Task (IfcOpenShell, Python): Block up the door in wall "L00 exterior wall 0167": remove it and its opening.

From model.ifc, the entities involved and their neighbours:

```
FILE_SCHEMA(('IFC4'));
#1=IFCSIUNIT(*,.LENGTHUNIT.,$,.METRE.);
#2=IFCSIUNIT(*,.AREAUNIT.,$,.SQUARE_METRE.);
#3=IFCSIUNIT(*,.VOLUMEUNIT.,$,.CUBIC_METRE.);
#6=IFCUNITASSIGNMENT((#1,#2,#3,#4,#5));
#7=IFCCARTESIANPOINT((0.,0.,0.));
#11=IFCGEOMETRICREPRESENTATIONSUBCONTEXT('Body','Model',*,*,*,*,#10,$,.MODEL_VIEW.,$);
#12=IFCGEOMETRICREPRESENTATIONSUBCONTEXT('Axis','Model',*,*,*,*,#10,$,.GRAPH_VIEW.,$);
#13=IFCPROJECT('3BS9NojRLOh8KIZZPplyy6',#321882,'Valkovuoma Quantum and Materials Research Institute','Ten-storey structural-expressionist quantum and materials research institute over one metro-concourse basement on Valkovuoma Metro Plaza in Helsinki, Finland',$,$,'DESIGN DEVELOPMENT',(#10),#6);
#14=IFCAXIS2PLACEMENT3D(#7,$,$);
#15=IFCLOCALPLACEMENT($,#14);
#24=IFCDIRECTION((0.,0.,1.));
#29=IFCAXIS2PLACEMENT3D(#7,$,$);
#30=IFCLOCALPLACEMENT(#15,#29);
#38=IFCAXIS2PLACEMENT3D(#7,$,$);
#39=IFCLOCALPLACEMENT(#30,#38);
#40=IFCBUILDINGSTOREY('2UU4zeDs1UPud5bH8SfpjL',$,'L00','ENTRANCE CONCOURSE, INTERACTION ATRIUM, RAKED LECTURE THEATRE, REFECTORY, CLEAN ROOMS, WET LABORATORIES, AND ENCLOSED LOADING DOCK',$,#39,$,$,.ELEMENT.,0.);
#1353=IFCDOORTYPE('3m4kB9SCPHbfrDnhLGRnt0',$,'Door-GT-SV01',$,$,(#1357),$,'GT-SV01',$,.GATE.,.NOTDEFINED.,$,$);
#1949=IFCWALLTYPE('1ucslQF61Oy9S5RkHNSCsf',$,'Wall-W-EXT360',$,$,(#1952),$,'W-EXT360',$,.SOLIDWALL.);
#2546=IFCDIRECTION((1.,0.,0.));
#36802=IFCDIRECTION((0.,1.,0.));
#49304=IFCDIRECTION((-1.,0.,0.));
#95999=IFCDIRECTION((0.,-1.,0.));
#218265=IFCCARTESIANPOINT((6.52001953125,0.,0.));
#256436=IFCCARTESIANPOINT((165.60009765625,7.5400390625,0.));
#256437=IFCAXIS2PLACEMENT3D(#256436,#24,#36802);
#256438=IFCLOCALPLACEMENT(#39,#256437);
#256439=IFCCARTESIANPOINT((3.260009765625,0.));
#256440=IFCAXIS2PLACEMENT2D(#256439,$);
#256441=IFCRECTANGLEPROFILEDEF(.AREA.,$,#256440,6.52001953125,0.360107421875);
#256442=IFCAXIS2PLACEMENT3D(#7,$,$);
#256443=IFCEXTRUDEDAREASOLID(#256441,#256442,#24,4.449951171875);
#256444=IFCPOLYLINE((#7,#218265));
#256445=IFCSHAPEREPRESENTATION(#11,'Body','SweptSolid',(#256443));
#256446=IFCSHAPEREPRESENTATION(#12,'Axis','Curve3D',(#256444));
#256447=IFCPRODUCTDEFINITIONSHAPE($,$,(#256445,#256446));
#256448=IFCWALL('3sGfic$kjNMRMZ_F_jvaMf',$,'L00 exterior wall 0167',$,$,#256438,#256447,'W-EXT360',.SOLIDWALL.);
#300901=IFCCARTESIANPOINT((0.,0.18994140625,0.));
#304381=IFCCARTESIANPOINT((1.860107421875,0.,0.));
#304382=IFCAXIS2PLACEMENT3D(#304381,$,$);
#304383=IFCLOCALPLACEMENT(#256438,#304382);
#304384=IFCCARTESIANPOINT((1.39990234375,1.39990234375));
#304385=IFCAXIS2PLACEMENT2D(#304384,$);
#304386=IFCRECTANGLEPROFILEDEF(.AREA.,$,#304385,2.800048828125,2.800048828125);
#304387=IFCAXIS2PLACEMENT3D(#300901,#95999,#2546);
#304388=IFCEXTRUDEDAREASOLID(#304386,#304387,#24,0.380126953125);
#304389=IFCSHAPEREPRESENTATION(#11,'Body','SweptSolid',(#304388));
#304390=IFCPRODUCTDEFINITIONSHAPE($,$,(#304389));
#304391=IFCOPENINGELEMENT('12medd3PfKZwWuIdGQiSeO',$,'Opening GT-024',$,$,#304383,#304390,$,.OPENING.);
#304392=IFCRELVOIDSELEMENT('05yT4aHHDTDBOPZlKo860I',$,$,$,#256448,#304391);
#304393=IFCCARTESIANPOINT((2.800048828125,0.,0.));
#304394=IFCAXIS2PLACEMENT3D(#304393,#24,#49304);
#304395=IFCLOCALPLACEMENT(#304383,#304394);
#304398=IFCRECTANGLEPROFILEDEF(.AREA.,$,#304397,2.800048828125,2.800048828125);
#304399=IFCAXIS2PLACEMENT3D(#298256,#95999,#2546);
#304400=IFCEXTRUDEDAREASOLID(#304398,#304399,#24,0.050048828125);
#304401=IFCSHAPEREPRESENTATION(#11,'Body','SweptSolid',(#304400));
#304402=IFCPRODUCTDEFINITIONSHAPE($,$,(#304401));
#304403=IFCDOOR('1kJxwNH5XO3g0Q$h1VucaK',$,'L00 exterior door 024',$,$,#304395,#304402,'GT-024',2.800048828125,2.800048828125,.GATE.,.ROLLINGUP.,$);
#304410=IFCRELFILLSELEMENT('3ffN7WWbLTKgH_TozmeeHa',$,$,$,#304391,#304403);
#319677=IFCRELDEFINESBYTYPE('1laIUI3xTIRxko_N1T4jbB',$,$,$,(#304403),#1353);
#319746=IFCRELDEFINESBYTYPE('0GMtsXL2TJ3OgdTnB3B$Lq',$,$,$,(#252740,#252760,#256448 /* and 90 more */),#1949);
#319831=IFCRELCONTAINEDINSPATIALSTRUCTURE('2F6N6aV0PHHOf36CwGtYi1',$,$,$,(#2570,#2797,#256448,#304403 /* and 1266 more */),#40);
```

```python
import ifcopenshell
import ifcopenshell.api.feature
import ifcopenshell.api.root
import ifcopenshell.geom
import ifcopenshell.util.shape

model = ifcopenshell.open("model.ifc")
settings = ifcopenshell.geom.settings()


def volume(element):
    """Net volume in cubic metres, openings subtracted."""
    shape = ifcopenshell.geom.create_shape(settings, element)
    return ifcopenshell.util.shape.get_volume(shape.geometry)


door = model.by_guid("1kJxwNH5XO3g0Q$h1VucaK")
opening = door.FillsVoids[0].RelatingOpeningElement
wall = opening.VoidsElements[0].RelatingBuildingElement
before = volume(wall)

ifcopenshell.api.root.remove_product(model, product=door)
ifcopenshell.api.feature.remove_feature(model, feature=opening)

after = volume(wall)

print(f"wall volume {before:.3f} -> {after:.3f} m3")

model.write("model-out.ifc")
```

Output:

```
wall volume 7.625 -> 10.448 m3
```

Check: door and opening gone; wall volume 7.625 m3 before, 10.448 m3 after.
